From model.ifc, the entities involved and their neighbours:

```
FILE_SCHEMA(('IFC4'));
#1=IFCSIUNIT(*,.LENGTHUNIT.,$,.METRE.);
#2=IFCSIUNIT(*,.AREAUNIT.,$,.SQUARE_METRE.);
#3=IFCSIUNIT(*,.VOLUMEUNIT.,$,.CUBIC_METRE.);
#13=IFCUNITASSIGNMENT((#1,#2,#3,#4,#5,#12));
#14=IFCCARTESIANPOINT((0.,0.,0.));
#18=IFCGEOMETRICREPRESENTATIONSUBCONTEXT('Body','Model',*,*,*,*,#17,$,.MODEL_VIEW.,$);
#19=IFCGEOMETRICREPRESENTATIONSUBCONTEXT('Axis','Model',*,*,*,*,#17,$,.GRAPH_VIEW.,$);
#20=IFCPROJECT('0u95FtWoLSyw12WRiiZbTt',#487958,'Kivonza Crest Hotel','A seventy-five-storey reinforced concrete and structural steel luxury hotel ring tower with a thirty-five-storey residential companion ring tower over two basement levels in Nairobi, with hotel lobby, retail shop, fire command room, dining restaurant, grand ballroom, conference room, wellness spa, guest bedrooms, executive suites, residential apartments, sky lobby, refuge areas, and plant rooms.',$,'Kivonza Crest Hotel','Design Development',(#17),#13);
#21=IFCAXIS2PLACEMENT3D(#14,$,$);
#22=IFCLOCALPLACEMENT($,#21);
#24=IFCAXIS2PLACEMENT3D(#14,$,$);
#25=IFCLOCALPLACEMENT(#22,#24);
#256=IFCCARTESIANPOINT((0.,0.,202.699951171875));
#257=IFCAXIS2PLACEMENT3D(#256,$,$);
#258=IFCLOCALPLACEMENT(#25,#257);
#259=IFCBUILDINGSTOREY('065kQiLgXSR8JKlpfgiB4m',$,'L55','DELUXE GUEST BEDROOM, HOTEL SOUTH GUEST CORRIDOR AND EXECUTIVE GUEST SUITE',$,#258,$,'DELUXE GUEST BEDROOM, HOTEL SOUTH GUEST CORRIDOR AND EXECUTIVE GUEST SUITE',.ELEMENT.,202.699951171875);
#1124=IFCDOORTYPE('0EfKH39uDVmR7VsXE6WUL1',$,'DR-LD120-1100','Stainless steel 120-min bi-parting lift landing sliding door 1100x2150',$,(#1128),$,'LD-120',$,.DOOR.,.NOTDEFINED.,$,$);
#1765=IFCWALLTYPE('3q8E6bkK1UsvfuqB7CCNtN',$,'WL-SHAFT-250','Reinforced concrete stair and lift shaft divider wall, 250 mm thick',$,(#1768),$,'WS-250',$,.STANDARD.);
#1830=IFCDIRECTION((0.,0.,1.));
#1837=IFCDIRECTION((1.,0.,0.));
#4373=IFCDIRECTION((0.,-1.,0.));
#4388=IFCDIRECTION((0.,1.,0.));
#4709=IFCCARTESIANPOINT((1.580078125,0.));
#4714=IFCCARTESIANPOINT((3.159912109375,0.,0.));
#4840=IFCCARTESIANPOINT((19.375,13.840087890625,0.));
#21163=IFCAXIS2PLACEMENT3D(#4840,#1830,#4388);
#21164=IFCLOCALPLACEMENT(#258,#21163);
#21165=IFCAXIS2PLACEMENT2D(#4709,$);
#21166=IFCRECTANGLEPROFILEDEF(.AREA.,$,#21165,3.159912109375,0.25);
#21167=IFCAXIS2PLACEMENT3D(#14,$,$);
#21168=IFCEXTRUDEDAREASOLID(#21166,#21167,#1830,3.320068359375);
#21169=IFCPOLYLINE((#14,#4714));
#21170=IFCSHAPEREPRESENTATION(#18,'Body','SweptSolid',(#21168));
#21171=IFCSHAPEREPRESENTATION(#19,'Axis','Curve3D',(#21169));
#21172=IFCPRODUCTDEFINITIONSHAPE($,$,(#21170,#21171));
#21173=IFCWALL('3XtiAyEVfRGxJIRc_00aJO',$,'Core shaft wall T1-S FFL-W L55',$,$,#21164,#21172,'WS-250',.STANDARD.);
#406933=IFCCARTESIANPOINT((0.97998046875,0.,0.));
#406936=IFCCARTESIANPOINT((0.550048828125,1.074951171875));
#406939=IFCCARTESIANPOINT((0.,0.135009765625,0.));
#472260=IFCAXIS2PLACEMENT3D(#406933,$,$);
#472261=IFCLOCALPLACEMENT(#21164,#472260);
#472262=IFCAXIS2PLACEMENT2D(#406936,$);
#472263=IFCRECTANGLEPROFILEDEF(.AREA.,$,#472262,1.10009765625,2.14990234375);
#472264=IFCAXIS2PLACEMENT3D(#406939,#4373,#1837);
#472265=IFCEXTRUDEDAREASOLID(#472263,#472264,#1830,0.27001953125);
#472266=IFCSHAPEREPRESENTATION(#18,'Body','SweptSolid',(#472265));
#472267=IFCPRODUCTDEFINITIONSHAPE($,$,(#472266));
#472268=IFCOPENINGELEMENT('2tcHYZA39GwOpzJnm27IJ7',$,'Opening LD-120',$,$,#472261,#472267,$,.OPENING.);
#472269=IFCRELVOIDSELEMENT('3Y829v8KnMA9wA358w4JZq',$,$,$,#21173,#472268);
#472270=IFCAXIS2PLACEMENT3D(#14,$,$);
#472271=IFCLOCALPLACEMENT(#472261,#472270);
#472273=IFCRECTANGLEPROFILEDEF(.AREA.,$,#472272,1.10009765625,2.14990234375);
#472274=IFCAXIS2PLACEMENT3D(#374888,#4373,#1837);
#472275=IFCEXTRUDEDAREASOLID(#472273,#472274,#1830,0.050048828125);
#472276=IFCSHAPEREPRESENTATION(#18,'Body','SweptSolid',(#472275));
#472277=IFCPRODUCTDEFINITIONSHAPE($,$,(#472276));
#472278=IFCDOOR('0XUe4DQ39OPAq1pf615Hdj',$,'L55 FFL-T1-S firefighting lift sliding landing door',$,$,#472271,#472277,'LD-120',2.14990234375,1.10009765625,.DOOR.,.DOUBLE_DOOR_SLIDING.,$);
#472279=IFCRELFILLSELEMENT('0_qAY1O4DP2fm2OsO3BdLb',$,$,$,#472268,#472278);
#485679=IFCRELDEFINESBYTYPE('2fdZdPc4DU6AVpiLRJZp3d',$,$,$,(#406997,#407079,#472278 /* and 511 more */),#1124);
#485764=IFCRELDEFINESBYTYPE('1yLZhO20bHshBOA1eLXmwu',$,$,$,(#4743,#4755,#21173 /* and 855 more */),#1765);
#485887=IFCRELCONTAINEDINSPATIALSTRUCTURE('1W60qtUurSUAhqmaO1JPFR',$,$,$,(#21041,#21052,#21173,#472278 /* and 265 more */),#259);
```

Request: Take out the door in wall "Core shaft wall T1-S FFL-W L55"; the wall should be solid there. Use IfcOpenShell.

```python
import ifcopenshell
import ifcopenshell.api.feature
import ifcopenshell.api.root
import ifcopenshell.geom
import ifcopenshell.util.shape

model = ifcopenshell.open("model.ifc")
settings = ifcopenshell.geom.settings()


def volume(element):
    """Net volume in cubic metres, openings subtracted."""
    shape = ifcopenshell.geom.create_shape(settings, element)
    return ifcopenshell.util.shape.get_volume(shape.geometry)


door = model.by_id(472278)
opening = door.FillsVoids[0].RelatingOpeningElement
wall = opening.VoidsElements[0].RelatingBuildingElement
before = volume(wall)

ifcopenshell.api.root.remove_product(model, product=door)
ifcopenshell.api.feature.remove_feature(model, feature=opening)

after = volume(wall)

print(f"wall volume {before:.3f} -> {after:.3f} m3")

model.write("model_updated.ifc")
```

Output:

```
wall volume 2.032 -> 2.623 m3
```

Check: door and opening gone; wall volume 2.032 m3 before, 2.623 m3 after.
